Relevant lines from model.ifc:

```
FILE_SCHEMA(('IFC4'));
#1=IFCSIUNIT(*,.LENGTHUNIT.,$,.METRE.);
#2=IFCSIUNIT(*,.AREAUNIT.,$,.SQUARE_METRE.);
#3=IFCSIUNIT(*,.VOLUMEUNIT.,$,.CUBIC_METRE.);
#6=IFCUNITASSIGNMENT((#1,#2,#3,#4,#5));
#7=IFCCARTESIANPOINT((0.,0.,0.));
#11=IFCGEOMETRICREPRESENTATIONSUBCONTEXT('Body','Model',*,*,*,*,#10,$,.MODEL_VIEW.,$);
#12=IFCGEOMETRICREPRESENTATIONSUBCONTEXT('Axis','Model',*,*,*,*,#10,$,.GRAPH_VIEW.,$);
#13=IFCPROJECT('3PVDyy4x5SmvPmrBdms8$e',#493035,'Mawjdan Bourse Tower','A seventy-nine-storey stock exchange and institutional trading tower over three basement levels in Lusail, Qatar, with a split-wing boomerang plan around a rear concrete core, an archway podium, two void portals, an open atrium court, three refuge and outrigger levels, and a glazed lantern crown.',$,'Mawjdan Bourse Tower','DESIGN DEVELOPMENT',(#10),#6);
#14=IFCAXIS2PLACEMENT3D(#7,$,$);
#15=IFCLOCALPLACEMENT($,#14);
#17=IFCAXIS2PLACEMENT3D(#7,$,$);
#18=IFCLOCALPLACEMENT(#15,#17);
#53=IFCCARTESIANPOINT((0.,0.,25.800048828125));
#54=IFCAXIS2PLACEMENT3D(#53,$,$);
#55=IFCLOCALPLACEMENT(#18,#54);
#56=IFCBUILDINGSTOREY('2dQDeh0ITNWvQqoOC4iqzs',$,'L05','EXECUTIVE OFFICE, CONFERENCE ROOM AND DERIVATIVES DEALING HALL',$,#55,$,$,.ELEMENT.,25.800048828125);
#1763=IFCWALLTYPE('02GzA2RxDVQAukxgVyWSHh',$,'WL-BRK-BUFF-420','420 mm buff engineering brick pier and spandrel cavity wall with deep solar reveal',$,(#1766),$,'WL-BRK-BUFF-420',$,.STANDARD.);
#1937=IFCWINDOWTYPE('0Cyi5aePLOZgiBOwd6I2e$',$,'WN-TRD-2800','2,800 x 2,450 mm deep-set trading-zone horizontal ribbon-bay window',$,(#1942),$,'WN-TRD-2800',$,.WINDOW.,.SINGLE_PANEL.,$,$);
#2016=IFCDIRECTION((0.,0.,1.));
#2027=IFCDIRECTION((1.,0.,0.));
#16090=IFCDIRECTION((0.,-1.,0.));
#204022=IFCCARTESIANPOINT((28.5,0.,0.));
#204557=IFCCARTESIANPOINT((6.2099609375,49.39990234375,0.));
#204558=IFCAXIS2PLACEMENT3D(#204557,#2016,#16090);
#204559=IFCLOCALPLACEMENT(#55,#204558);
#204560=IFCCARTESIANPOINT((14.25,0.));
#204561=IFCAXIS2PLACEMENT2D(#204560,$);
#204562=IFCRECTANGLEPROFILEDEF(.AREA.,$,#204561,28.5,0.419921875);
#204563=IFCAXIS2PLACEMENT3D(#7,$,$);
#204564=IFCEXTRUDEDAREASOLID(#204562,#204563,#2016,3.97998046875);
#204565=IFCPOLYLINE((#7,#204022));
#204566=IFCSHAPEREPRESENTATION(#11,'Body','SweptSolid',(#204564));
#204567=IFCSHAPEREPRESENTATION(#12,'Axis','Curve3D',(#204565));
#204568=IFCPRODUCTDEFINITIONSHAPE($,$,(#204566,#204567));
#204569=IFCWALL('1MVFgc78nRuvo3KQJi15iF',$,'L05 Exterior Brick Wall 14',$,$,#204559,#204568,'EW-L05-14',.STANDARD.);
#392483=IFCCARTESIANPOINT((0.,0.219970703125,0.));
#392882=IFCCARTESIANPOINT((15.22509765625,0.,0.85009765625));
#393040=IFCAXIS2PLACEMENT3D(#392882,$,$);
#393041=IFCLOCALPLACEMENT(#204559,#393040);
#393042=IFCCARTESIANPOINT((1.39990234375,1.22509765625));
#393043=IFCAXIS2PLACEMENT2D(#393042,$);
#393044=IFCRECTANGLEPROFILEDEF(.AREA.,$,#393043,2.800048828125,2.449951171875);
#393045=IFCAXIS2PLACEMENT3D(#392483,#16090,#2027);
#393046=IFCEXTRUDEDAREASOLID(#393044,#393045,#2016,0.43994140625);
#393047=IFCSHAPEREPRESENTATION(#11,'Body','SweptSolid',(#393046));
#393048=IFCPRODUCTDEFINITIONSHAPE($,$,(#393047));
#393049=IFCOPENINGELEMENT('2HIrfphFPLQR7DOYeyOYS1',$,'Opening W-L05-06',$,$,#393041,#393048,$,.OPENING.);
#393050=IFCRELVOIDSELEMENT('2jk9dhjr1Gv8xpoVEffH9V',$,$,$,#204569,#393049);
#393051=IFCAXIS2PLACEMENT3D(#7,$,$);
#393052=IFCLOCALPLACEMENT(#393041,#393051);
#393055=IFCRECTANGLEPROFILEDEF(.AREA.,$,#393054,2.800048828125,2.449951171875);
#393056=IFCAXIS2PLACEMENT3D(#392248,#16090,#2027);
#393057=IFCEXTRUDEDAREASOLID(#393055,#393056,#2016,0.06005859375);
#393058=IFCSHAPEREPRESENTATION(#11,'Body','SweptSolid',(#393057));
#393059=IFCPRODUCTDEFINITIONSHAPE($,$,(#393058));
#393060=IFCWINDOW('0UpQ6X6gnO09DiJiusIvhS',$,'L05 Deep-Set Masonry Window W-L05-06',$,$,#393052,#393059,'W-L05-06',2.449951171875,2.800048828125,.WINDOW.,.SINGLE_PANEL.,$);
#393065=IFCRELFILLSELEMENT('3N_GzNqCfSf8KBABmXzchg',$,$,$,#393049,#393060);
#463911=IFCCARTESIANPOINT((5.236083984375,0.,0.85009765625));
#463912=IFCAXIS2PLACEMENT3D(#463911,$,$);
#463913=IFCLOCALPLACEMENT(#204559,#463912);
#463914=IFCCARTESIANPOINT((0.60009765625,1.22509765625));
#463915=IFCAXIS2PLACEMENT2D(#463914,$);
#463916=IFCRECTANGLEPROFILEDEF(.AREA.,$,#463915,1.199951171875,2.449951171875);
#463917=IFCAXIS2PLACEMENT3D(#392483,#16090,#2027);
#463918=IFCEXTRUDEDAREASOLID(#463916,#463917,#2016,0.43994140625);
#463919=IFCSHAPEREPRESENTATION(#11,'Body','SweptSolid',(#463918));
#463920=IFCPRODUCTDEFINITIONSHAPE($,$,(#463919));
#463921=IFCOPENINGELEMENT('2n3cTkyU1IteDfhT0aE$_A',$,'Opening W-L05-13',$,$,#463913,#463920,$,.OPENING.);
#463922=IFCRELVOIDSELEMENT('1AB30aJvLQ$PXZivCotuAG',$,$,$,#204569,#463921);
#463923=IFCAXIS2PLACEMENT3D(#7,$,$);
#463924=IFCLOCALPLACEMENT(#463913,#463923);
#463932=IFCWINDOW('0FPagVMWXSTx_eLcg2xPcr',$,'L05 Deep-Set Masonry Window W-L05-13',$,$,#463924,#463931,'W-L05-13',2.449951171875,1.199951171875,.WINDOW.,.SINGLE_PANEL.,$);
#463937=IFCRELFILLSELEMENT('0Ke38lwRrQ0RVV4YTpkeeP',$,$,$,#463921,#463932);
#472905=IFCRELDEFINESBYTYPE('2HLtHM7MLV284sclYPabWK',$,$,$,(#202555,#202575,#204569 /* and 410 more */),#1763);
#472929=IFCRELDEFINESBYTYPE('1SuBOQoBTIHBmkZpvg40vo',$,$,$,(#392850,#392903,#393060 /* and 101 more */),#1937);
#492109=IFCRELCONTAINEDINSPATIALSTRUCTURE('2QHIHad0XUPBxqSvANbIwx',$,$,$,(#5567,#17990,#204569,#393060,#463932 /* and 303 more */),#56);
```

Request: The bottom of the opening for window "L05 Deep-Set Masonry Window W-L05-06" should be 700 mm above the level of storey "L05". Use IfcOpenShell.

```python
import numpy as np
import ifcopenshell
import ifcopenshell.api.geometry
import ifcopenshell.geom
import ifcopenshell.util.element
import ifcopenshell.util.placement
import ifcopenshell.util.shape
import ifcopenshell.util.unit

model = ifcopenshell.open("model.ifc")
unit_scale = ifcopenshell.util.unit.calculate_unit_scale(model)

window = model.by_guid("0UpQ6X6gnO09DiJiusIvhS")
opening = window.FillsVoids[0].RelatingOpeningElement
storey = ifcopenshell.util.element.get_container(window, ifc_class="IfcBuildingStorey")
level = ifcopenshell.util.placement.get_local_placement(storey.ObjectPlacement)[2, 3]

# The opening's origin need not be at the sill, so measure its lowest point.
shape = ifcopenshell.geom.create_shape(ifcopenshell.geom.settings(), opening)
bottom = ifcopenshell.util.shape.get_shape_bottom_elevation(shape, shape.geometry) / unit_scale
dz = level + 0.7 / unit_scale - bottom

shift = np.array([0.0, 0.0, dz])
# The window is placed relative to its opening, so it follows when the opening moves.
matrix = ifcopenshell.util.placement.get_local_placement(opening.ObjectPlacement)
matrix[:3, 3] += shift
ifcopenshell.api.geometry.edit_object_placement(
    model, product=opening, matrix=matrix, is_si=False, should_transform_children=True
)

print(f"moved by {dz * unit_scale:+.3f} m")

model.write("model_edited.ifc")
```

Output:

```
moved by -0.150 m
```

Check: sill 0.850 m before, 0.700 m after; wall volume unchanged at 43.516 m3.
